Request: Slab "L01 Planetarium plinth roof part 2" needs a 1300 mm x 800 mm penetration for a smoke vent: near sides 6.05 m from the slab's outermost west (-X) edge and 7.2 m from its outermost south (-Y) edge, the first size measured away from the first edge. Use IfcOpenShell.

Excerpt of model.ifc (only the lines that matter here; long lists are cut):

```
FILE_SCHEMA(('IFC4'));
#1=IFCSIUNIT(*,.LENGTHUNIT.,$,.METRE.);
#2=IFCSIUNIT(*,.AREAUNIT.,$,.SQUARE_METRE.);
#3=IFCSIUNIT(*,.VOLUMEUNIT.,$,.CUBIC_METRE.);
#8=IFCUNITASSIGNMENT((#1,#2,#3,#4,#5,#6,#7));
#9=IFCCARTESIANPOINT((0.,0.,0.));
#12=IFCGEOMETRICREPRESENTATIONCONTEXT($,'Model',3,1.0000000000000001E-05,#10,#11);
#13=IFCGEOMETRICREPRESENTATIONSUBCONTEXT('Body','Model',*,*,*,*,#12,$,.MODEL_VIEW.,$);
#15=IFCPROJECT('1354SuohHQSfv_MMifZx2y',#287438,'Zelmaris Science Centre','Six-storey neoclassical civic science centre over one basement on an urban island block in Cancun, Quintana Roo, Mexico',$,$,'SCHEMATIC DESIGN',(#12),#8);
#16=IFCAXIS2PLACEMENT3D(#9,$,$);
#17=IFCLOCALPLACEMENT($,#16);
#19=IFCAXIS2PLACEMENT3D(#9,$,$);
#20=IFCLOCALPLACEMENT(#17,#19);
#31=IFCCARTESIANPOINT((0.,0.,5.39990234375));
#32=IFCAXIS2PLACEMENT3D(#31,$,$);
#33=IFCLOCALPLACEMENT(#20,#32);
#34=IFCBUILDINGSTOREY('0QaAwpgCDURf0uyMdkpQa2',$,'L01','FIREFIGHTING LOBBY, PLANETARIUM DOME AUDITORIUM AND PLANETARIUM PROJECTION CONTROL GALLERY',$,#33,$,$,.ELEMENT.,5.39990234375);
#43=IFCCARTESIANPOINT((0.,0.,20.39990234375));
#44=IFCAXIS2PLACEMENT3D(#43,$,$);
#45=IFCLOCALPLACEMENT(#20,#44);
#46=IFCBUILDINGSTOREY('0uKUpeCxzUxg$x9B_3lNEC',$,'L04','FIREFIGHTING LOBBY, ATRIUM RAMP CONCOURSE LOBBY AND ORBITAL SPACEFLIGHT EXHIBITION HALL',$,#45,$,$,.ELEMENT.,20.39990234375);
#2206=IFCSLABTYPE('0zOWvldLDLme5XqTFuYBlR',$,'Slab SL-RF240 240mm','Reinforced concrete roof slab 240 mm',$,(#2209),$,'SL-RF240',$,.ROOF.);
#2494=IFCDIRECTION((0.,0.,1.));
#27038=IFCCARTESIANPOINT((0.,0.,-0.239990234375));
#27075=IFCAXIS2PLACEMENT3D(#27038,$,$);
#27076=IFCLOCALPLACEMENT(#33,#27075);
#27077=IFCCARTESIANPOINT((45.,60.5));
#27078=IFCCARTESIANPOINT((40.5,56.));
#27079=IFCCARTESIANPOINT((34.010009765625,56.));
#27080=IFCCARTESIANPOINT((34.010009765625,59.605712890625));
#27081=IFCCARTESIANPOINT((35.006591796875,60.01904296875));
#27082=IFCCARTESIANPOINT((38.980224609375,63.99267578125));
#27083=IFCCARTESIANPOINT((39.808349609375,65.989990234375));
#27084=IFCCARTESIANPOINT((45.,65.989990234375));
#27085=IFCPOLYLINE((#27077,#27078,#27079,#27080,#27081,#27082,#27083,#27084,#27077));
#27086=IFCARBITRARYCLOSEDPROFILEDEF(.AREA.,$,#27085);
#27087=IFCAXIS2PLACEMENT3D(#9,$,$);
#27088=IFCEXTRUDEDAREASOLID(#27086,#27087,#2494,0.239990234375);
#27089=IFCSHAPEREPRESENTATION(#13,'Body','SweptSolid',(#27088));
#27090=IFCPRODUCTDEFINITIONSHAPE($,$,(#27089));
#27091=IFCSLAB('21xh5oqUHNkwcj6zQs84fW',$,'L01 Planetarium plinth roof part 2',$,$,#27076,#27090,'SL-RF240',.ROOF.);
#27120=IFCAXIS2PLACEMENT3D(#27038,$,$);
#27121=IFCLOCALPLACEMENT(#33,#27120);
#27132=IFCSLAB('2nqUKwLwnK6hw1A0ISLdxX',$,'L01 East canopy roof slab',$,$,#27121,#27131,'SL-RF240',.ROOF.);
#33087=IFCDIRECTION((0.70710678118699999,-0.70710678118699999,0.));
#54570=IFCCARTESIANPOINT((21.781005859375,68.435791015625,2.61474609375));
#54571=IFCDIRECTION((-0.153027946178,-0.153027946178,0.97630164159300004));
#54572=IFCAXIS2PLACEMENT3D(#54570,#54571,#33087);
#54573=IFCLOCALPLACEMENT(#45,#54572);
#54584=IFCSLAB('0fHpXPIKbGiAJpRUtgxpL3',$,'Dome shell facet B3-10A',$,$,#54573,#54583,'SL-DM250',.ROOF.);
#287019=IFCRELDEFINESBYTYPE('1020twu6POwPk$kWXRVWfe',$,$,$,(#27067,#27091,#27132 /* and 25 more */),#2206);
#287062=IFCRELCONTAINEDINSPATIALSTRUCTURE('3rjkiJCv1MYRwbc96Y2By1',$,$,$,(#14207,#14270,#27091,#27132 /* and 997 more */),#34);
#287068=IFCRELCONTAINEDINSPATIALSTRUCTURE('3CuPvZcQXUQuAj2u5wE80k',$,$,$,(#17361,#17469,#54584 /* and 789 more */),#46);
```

```python
import numpy as np
import ifcopenshell
import ifcopenshell.api.feature
import ifcopenshell.api.geometry
import ifcopenshell.api.root
import ifcopenshell.geom
import ifcopenshell.util.placement
import ifcopenshell.util.representation
import ifcopenshell.util.shape
import ifcopenshell.util.unit

model = ifcopenshell.open("model.ifc")
unit_scale = ifcopenshell.util.unit.calculate_unit_scale(model)
settings = ifcopenshell.geom.settings()


def volume(element):
    """Net volume in cubic metres, openings subtracted."""
    shape = ifcopenshell.geom.create_shape(settings, element)
    return ifcopenshell.util.shape.get_volume(shape.geometry)


slab = model.by_guid("21xh5oqUHNkwcj6zQs84fW")
before = volume(slab)

# Extent in the slab's own axes, in metres. The edges named are its -X and -Y sides.
slab_shape = ifcopenshell.geom.create_shape(settings, slab)
vertices = ifcopenshell.util.shape.get_vertices(slab_shape.geometry)
x_min, y_min, bottom = vertices.min(axis=0)
top = vertices[:, 2].max()

opening = ifcopenshell.api.root.create_entity(model, ifc_class="IfcOpeningElement", name="Smoke vent opening", predefined_type="OPENING")
context = ifcopenshell.util.representation.get_context(model, "Model", "Body", "MODEL_VIEW")
width, depth = 1.3, 0.8
outline = [(0.0, 0.0), (width, 0.0), (width, depth), (0.0, depth), (0.0, 0.0)]
# Overshoot both faces by 50 mm so the cut is clean.
shape = ifcopenshell.api.geometry.add_slab_representation(
    model, context=context, depth=top - bottom + 0.1, polyline=outline
)
ifcopenshell.api.geometry.assign_representation(model, product=opening, representation=shape)

matrix = ifcopenshell.util.placement.get_local_placement(slab.ObjectPlacement)
matrix[:, 3] = matrix @ np.append(np.array([x_min + 6.05, y_min + 7.2, bottom - 0.05]) / unit_scale, 1.0)
ifcopenshell.api.geometry.edit_object_placement(model, product=opening, matrix=matrix, is_si=False)
ifcopenshell.api.feature.add_feature(model, feature=opening, element=slab)

after = volume(slab)

print(f"slab volume {before:.3f} -> {after:.3f} m3")

model.write("model_v2.ifc")
```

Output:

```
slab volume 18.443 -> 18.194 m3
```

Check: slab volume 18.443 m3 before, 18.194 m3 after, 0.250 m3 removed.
